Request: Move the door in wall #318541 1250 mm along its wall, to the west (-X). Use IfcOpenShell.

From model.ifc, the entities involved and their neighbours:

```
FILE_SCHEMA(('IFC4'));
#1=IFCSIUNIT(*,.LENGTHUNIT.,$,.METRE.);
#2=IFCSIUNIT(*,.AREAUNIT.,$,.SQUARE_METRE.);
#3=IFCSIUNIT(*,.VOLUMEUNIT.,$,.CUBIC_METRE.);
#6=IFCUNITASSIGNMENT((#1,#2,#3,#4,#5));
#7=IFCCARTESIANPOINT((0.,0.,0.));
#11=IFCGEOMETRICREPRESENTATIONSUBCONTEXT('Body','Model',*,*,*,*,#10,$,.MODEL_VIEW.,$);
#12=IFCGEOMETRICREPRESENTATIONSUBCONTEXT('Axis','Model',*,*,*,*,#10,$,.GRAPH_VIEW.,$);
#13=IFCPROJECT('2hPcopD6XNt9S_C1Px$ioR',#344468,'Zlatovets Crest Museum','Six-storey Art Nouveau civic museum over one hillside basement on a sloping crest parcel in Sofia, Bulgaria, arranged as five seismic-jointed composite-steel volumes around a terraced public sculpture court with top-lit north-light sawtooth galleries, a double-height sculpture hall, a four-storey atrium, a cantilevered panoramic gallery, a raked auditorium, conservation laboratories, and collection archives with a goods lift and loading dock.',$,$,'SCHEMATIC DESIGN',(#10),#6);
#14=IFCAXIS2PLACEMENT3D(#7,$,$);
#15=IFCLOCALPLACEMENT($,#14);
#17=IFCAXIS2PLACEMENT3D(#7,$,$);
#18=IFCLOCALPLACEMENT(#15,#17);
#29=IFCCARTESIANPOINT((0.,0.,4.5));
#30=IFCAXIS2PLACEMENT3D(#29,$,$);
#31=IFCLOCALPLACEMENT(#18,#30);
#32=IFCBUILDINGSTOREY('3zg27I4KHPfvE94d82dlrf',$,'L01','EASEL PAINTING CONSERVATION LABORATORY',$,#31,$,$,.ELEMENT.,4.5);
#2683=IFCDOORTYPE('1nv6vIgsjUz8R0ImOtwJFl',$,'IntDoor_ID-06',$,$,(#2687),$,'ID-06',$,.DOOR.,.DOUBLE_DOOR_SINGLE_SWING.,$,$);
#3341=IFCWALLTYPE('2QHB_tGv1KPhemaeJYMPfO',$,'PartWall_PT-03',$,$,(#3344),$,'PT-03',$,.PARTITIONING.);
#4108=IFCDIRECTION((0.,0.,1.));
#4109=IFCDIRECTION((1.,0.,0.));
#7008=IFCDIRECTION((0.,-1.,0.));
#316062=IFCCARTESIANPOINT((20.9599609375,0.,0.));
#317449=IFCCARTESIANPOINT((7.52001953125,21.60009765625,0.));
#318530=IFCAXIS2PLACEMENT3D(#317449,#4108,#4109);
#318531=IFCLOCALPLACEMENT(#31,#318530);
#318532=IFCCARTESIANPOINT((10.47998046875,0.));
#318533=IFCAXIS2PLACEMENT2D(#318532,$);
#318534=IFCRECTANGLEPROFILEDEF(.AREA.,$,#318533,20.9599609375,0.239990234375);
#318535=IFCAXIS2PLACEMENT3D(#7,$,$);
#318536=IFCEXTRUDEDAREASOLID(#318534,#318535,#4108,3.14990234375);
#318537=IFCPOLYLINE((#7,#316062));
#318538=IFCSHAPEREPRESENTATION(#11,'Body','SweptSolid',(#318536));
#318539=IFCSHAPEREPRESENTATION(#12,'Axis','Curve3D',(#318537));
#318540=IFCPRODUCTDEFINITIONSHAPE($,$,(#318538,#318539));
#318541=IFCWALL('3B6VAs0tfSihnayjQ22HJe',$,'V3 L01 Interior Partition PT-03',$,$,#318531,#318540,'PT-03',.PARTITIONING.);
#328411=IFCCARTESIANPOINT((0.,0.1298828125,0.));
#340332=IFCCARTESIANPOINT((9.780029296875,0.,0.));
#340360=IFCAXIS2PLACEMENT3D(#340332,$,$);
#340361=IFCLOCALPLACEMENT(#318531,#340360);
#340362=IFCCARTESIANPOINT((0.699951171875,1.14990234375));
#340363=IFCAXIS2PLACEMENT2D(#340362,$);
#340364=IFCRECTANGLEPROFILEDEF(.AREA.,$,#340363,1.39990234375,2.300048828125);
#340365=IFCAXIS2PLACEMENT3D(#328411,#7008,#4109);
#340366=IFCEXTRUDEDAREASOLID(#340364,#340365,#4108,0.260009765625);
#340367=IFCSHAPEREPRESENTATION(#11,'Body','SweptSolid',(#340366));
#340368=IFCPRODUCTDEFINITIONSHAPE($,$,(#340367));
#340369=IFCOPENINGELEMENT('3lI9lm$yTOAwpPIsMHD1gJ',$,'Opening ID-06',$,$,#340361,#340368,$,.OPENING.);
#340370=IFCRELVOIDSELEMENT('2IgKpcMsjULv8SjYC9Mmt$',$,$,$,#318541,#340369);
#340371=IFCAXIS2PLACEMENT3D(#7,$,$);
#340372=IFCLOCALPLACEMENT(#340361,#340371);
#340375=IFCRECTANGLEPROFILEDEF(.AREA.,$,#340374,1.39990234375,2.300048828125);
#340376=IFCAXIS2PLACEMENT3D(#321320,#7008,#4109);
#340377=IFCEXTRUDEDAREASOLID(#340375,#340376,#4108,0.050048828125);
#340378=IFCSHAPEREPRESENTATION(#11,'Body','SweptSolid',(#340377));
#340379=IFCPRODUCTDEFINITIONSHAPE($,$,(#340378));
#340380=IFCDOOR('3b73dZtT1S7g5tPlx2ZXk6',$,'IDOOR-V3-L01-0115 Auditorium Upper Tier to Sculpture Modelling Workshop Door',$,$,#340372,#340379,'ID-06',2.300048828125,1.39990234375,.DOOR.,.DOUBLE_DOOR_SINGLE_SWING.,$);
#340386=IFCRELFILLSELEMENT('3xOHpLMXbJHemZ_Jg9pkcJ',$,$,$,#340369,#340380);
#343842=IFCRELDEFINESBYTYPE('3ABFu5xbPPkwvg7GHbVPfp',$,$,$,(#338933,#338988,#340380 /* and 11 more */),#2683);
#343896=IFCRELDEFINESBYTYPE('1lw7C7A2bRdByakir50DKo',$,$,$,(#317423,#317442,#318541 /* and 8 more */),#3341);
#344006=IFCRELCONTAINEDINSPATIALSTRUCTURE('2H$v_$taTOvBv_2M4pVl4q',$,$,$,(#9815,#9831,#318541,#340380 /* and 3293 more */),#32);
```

```python
import ifcopenshell
import ifcopenshell.api.geometry
import ifcopenshell.util.placement
import ifcopenshell.util.unit

model = ifcopenshell.open("model.ifc")
unit_scale = ifcopenshell.util.unit.calculate_unit_scale(model)

door = model.by_id(340380)
opening = door.FillsVoids[0].RelatingOpeningElement
wall = opening.VoidsElements[0].RelatingBuildingElement

wall_matrix = ifcopenshell.util.placement.get_local_placement(wall.ObjectPlacement)
shift = wall_matrix[:3, 0] * -1.25 / unit_scale
before = ifcopenshell.util.placement.get_local_placement(door.ObjectPlacement)[:3, 3].copy()

# The door is placed relative to its opening, so it follows when the opening moves.
matrix = ifcopenshell.util.placement.get_local_placement(opening.ObjectPlacement)
matrix[:3, 3] += shift
ifcopenshell.api.geometry.edit_object_placement(
    model, product=opening, matrix=matrix, is_si=False, should_transform_children=True
)

after = ifcopenshell.util.placement.get_local_placement(door.ObjectPlacement)[:3, 3]
print("door moved by", (after - before).round(3) + 0.0)

model.write("model_rev.ifc")
```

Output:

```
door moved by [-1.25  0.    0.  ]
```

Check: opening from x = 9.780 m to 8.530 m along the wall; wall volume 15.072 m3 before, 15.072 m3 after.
